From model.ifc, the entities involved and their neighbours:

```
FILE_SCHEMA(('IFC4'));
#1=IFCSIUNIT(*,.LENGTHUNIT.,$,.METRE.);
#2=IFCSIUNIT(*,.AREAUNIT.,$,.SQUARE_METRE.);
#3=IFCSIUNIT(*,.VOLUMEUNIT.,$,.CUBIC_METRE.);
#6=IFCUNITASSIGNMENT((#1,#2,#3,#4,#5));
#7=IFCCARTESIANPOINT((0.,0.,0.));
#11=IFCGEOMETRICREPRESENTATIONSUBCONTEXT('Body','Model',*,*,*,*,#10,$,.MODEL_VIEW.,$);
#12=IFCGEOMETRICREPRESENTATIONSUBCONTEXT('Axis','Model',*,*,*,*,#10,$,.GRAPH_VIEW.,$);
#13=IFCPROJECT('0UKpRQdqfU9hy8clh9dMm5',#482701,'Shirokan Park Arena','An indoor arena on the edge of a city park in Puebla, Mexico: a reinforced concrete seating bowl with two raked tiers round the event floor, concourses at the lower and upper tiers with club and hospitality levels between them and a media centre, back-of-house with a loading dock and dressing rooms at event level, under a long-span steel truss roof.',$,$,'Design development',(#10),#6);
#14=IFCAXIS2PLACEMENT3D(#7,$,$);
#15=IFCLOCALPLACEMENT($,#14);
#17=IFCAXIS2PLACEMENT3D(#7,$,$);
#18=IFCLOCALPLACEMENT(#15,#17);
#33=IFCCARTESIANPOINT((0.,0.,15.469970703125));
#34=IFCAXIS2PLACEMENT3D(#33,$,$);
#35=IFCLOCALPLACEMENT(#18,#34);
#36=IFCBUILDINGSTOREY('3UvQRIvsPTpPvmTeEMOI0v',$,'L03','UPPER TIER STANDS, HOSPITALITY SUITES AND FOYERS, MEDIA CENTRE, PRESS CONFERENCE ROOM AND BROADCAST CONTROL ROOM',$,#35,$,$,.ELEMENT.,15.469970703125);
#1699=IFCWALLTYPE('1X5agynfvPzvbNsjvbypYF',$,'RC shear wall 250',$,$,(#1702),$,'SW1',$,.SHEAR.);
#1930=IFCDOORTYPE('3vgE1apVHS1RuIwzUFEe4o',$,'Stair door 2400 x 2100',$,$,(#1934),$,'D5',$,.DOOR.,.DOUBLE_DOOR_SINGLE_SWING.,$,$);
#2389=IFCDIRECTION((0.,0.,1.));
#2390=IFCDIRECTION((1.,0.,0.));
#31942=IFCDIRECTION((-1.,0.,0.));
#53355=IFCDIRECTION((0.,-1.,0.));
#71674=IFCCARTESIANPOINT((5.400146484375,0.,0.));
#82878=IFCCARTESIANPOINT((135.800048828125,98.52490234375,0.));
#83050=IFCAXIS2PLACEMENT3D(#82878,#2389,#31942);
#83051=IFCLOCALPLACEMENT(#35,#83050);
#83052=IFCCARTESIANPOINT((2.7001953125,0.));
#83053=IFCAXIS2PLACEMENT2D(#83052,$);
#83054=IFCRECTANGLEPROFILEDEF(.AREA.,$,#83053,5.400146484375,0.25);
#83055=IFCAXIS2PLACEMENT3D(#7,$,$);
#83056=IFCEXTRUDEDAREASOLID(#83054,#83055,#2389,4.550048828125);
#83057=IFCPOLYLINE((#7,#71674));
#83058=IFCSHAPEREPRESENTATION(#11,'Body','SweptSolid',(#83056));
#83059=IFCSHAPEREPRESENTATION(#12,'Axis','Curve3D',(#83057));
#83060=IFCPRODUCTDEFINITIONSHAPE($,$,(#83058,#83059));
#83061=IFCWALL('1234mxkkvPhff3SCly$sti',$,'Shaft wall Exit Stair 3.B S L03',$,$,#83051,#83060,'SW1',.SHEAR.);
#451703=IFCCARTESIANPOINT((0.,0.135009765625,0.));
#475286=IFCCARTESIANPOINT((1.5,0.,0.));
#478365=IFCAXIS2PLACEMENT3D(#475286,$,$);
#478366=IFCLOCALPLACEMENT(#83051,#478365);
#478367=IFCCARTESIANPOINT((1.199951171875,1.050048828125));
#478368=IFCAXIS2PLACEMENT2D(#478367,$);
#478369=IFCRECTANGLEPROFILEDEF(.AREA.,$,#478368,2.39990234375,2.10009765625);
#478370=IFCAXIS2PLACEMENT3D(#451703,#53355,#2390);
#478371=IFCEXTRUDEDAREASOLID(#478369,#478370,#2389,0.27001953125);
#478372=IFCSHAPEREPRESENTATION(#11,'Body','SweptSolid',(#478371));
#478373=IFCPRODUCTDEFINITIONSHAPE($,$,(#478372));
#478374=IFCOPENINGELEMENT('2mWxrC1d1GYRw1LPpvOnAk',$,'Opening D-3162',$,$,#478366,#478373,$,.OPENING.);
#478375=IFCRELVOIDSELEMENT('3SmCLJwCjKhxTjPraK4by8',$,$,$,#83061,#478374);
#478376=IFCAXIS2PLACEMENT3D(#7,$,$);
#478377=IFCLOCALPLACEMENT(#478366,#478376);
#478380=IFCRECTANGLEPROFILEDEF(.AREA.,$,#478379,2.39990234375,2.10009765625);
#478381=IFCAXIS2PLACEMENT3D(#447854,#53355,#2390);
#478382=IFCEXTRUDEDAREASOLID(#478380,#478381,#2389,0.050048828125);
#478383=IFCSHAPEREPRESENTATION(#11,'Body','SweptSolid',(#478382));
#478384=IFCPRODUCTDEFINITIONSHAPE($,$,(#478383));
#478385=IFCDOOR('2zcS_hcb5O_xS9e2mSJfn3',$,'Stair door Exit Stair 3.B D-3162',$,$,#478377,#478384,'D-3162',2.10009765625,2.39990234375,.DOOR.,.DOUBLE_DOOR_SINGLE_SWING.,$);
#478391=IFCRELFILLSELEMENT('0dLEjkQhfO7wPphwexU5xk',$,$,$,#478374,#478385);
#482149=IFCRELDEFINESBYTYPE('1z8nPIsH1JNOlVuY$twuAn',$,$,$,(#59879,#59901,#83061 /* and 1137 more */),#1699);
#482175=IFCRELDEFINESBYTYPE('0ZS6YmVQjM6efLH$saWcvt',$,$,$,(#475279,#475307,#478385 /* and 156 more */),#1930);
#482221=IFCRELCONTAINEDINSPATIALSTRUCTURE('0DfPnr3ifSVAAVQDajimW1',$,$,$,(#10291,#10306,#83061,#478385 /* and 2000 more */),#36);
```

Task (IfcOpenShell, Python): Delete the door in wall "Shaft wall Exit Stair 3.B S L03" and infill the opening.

```python
import ifcopenshell
import ifcopenshell.api.feature
import ifcopenshell.api.root
import ifcopenshell.geom
import ifcopenshell.util.shape

model = ifcopenshell.open("model.ifc")
settings = ifcopenshell.geom.settings()


def volume(element):
    """Net volume in cubic metres, openings subtracted."""
    shape = ifcopenshell.geom.create_shape(settings, element)
    return ifcopenshell.util.shape.get_volume(shape.geometry)


door = model.by_guid("2zcS_hcb5O_xS9e2mSJfn3")
opening = door.FillsVoids[0].RelatingOpeningElement
wall = opening.VoidsElements[0].RelatingBuildingElement
before = volume(wall)

ifcopenshell.api.root.remove_product(model, product=door)
ifcopenshell.api.feature.remove_feature(model, feature=opening)

after = volume(wall)

print(f"wall volume {before:.3f} -> {after:.3f} m3")

model.write("model_edited.ifc")
```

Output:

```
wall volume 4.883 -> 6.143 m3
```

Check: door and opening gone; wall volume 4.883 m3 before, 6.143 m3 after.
